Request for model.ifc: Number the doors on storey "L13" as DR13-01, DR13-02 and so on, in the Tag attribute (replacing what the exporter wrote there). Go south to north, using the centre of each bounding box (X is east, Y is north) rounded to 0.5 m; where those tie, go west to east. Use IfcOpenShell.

First a look at what the model holds.

```python
import ifcopenshell
import ifcopenshell.util.element
import ifcopenshell.util.placement

model = ifcopenshell.open("model.ifc")
print(model.schema)
storey = next(s for s in model.by_type("IfcBuildingStorey") if s.Name == "L13")
doors = [e for e in ifcopenshell.util.element.get_decomposition(storey) if e.is_a("IfcDoor")]
for e in sorted(doors, key=lambda e: e.id()):
    origin = ifcopenshell.util.placement.get_local_placement(e.ObjectPlacement)[:3, 3]
    print(e.id(), e.Tag, e.Name, origin.round(2) + 0.0, sep=" | ")
```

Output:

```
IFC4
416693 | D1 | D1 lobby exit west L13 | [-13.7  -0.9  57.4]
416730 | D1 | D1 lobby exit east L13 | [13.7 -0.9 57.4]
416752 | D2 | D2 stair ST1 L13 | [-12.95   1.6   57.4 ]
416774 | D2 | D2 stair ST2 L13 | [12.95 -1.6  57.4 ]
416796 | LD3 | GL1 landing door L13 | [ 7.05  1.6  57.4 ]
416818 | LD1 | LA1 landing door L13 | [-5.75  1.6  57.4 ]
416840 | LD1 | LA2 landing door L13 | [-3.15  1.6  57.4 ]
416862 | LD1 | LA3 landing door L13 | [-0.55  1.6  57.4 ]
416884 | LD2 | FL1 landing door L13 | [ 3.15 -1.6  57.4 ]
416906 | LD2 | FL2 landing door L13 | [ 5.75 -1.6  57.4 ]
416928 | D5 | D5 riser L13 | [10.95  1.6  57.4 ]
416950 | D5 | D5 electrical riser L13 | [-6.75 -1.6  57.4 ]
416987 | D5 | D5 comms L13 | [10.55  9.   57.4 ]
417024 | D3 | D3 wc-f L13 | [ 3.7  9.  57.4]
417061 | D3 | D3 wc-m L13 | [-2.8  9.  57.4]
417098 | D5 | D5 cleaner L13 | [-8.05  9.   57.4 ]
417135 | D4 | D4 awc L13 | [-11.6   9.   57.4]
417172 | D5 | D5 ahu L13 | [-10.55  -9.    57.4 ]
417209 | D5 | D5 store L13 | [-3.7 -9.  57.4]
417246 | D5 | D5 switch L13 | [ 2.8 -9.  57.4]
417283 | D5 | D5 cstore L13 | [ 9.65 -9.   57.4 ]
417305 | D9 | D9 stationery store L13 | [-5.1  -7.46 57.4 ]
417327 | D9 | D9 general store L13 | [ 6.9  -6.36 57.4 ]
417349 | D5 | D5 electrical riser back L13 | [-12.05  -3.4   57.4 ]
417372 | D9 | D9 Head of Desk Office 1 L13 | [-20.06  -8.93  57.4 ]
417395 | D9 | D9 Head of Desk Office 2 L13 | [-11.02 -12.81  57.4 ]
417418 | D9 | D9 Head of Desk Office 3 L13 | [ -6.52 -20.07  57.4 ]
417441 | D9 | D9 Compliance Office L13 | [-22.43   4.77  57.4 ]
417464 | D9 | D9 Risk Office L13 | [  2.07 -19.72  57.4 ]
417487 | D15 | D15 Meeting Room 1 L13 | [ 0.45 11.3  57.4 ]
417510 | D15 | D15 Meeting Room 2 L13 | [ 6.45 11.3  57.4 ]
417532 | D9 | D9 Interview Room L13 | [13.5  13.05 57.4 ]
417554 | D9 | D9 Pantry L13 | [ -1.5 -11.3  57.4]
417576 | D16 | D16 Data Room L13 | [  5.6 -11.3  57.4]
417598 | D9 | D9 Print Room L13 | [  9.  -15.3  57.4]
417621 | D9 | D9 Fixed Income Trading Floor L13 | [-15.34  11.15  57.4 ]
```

```python
import ifcopenshell
import ifcopenshell.geom
import ifcopenshell.util.element
import ifcopenshell.util.shape

model = ifcopenshell.open("model.ifc")
settings = ifcopenshell.geom.settings()
settings.set("use-world-coords", True)


def centre(element):
    shape = ifcopenshell.geom.create_shape(settings, element)
    return ifcopenshell.util.shape.get_bbox_centroid(shape.geometry)


storey = next(s for s in model.by_type("IfcBuildingStorey") if s.Name == "L13")
doors = [e for e in ifcopenshell.util.element.get_decomposition(storey) if e.is_a("IfcDoor")]

# Insertion points can sit at a corner or the storey origin, so sort by the geometry (in metres).
centres = {e: centre(e) for e in doors}
doors.sort(key=lambda e: (round(centres[e][1] / 0.5), centres[e][0]))

for i, e in enumerate(doors, start=1):
    number = f"DR13-{i:02d}"
    e.Tag = number
    print(e.id(), number)

model.write("model_edited.ifc")
```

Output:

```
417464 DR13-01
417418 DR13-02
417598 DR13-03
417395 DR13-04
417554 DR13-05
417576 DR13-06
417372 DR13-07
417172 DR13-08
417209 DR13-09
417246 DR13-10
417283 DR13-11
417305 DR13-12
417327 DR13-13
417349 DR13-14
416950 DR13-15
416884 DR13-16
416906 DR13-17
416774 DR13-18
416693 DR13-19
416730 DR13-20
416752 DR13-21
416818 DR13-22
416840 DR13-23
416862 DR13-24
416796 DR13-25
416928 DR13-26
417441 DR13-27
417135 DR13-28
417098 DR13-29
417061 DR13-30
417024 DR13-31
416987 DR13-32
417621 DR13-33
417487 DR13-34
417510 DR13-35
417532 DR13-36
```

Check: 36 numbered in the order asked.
